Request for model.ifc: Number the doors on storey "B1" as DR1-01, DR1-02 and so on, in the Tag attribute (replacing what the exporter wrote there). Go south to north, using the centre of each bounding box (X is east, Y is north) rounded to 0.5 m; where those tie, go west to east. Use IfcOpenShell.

First a look at what the model holds.

```python
import ifcopenshell
import ifcopenshell.util.element
import ifcopenshell.util.placement

model = ifcopenshell.open("model.ifc")
print(model.schema)
storey = next(s for s in model.by_type("IfcBuildingStorey") if s.Name == "B1")
doors = [e for e in ifcopenshell.util.element.get_decomposition(storey) if e.is_a("IfcDoor")]
for e in sorted(doors, key=lambda e: e.id()):
    origin = ifcopenshell.util.placement.get_local_placement(e.ObjectPlacement)[:3, 3]
    print(e.id(), e.Tag, e.Name, origin.round(2) + 0.0, sep=" | ")
```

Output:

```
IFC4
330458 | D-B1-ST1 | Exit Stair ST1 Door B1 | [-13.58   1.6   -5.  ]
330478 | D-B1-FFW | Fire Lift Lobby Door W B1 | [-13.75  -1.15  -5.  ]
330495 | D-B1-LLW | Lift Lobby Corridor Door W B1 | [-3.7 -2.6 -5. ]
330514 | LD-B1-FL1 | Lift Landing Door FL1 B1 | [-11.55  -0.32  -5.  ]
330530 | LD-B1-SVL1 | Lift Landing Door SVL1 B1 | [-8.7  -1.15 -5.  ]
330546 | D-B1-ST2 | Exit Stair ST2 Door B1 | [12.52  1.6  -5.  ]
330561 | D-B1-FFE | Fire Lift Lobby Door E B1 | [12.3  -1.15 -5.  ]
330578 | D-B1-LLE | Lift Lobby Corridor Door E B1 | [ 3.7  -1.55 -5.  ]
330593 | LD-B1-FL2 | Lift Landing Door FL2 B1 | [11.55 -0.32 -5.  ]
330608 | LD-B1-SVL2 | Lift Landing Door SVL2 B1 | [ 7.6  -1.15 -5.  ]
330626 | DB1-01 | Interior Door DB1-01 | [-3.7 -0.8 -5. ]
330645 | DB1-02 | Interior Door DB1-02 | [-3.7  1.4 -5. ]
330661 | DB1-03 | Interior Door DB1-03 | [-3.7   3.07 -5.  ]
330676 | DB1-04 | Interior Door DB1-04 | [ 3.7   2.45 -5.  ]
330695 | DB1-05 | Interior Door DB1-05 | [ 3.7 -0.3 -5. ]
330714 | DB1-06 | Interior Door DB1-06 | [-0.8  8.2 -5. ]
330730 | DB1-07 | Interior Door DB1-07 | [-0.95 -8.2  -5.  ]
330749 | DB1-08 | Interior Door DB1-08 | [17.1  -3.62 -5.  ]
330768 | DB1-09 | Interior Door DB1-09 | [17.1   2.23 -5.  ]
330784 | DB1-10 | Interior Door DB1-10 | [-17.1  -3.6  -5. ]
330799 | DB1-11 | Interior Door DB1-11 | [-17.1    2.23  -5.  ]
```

```python
import ifcopenshell
import ifcopenshell.geom
import ifcopenshell.util.element
import ifcopenshell.util.shape

model = ifcopenshell.open("model.ifc")
settings = ifcopenshell.geom.settings()
settings.set("use-world-coords", True)


def centre(element):
    shape = ifcopenshell.geom.create_shape(settings, element)
    return ifcopenshell.util.shape.get_bbox_centroid(shape.geometry)


storey = next(s for s in model.by_type("IfcBuildingStorey") if s.Name == "B1")
doors = [e for e in ifcopenshell.util.element.get_decomposition(storey) if e.is_a("IfcDoor")]

# Insertion points can sit at a corner or the storey origin, so sort by the geometry (in metres).
centres = {e: centre(e) for e in doors}
doors.sort(key=lambda e: (round(centres[e][1] / 0.5), centres[e][0]))

for i, e in enumerate(doors, start=1):
    number = f"DR1-{i:02d}"
    e.Tag = number
    print(e.id(), number)

model.write("model_edited.ifc")
```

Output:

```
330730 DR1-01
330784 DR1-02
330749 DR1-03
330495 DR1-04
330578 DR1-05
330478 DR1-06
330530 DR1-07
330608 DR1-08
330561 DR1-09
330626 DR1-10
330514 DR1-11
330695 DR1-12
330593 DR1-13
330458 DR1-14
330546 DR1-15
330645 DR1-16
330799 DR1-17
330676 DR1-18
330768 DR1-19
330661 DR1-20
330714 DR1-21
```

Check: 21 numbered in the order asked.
